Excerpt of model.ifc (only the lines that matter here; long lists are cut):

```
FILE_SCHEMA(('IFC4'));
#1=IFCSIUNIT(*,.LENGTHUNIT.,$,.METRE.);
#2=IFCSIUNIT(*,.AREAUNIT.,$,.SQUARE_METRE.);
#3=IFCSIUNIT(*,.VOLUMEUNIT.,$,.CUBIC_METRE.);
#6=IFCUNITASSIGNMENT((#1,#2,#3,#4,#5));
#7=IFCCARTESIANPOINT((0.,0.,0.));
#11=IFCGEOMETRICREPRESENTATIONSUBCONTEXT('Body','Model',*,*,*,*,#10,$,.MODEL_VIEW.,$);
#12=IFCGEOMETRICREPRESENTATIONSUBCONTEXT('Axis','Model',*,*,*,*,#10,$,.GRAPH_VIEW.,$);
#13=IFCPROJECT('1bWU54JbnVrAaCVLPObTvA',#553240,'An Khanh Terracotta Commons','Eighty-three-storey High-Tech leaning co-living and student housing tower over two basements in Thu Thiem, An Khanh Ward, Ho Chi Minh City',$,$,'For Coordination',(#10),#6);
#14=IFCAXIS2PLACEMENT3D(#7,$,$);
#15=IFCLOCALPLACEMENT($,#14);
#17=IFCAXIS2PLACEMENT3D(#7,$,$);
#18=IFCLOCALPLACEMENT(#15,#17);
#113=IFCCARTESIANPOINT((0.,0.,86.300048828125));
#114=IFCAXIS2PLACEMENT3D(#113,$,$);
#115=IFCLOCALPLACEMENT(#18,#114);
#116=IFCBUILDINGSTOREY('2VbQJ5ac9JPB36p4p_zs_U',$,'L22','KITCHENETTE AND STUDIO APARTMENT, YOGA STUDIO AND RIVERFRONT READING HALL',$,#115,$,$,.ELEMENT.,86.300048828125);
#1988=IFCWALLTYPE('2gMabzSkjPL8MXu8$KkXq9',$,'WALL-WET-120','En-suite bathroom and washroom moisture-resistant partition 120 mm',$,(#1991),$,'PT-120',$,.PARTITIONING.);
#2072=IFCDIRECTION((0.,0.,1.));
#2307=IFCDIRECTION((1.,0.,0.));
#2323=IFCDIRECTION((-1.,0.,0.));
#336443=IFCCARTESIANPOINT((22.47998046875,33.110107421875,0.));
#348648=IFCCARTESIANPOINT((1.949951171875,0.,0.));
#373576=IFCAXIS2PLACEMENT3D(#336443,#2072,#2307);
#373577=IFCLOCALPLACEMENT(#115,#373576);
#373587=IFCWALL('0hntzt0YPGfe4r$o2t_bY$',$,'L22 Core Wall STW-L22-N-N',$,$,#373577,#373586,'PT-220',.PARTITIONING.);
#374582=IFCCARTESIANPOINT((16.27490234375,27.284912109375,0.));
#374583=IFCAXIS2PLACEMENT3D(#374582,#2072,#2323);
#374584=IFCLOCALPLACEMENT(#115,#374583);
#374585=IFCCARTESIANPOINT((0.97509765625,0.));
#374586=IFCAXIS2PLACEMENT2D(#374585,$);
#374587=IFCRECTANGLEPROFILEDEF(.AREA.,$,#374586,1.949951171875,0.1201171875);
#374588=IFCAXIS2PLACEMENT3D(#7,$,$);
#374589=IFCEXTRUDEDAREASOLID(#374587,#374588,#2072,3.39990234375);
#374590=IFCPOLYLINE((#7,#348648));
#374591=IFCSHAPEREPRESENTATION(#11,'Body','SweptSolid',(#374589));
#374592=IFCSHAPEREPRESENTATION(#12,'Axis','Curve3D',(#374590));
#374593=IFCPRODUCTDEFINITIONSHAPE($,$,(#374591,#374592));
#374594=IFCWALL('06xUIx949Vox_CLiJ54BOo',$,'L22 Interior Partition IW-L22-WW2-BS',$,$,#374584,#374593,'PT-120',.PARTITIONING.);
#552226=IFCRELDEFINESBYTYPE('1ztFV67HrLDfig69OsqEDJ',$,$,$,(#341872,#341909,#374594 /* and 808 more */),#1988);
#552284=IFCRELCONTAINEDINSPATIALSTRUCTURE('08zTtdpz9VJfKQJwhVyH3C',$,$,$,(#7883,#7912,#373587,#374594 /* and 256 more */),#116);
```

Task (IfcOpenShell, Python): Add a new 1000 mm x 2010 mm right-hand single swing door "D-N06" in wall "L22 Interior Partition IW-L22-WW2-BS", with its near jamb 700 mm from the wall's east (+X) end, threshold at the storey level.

```python
import numpy as np
import ifcopenshell
import ifcopenshell.api.feature
import ifcopenshell.api.geometry
import ifcopenshell.api.root
import ifcopenshell.api.spatial
import ifcopenshell.geom
import ifcopenshell.util.element
import ifcopenshell.util.placement
import ifcopenshell.util.representation
import ifcopenshell.util.shape
import ifcopenshell.util.unit

model = ifcopenshell.open("model.ifc")
unit_scale = ifcopenshell.util.unit.calculate_unit_scale(model)
settings = ifcopenshell.geom.settings()


def volume(element):
    """Net volume in cubic metres, openings subtracted."""
    shape = ifcopenshell.geom.create_shape(settings, element)
    return ifcopenshell.util.shape.get_volume(shape.geometry)


wall = model.by_guid("06xUIx949Vox_CLiJ54BOo")
storey = ifcopenshell.util.element.get_container(wall, ifc_class="IfcBuildingStorey")
context = ifcopenshell.util.representation.get_context(model, "Model", "Body", "MODEL_VIEW")
before = volume(wall)

width, height, from_end, sill = 1, 2.01, 0.7, 0.0  # metres

# The wall runs along its own X axis, and the end named is its -X end.
wall_shape = ifcopenshell.geom.create_shape(settings, wall)
x, y, z = ifcopenshell.util.shape.get_vertices(wall_shape.geometry).T
start = x.min() + from_end
face, thickness = float(y.min()), float(y.max() - y.min())
wall_matrix = ifcopenshell.util.placement.get_local_placement(wall.ObjectPlacement)
level = ifcopenshell.util.placement.get_local_placement(storey.ObjectPlacement)[2, 3]


def in_wall(x, y):
    """Placement at x, y metres in the wall's axes, at sill height."""
    matrix = wall_matrix.copy()
    matrix[:, 3] = wall_matrix @ np.array([x / unit_scale, y / unit_scale, 0.0, 1.0])
    matrix[2, 3] = level + sill / unit_scale
    return matrix


# Opening: a box that overshoots both wall faces by 50 mm.
opening = ifcopenshell.api.root.create_entity(model, ifc_class="IfcOpeningElement", predefined_type="OPENING")
box = ifcopenshell.api.geometry.add_wall_representation(
    model, context=context, length=width, height=height, thickness=thickness + 0.1
)
ifcopenshell.api.geometry.assign_representation(model, product=opening, representation=box)
ifcopenshell.api.geometry.edit_object_placement(model, product=opening, matrix=in_wall(start, face - 0.05), is_si=False)
ifcopenshell.api.feature.add_feature(model, feature=opening, element=wall)

door = ifcopenshell.api.root.create_entity(model, ifc_class="IfcDoor", name="D-N06", predefined_type="DOOR")
door.OverallWidth, door.OverallHeight = width / unit_scale, height / unit_scale
door.OperationType = "SINGLE_SWING_RIGHT"
body = ifcopenshell.api.geometry.add_door_representation(
    model,
    context=context,
    overall_width=door.OverallWidth,
    overall_height=door.OverallHeight,
    operation_type="SINGLE_SWING_RIGHT",
    lining_properties={"LiningDepth": thickness / unit_scale, "ThresholdDepth": thickness / unit_scale},
)
ifcopenshell.api.geometry.assign_representation(model, product=door, representation=body)
ifcopenshell.api.spatial.assign_container(model, products=[door], relating_structure=storey)
ifcopenshell.api.feature.add_filling(model, opening=opening, element=door)

# The lining spans the wall, so the door starts at the wall face.
ifcopenshell.api.geometry.edit_object_placement(model, product=door, matrix=in_wall(start, face), is_si=False)

after = volume(wall)

print(f"wall volume {before:.3f} -> {after:.3f} m3")

model.write("model_updated.ifc")
```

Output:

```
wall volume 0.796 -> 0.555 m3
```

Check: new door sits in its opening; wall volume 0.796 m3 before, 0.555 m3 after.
